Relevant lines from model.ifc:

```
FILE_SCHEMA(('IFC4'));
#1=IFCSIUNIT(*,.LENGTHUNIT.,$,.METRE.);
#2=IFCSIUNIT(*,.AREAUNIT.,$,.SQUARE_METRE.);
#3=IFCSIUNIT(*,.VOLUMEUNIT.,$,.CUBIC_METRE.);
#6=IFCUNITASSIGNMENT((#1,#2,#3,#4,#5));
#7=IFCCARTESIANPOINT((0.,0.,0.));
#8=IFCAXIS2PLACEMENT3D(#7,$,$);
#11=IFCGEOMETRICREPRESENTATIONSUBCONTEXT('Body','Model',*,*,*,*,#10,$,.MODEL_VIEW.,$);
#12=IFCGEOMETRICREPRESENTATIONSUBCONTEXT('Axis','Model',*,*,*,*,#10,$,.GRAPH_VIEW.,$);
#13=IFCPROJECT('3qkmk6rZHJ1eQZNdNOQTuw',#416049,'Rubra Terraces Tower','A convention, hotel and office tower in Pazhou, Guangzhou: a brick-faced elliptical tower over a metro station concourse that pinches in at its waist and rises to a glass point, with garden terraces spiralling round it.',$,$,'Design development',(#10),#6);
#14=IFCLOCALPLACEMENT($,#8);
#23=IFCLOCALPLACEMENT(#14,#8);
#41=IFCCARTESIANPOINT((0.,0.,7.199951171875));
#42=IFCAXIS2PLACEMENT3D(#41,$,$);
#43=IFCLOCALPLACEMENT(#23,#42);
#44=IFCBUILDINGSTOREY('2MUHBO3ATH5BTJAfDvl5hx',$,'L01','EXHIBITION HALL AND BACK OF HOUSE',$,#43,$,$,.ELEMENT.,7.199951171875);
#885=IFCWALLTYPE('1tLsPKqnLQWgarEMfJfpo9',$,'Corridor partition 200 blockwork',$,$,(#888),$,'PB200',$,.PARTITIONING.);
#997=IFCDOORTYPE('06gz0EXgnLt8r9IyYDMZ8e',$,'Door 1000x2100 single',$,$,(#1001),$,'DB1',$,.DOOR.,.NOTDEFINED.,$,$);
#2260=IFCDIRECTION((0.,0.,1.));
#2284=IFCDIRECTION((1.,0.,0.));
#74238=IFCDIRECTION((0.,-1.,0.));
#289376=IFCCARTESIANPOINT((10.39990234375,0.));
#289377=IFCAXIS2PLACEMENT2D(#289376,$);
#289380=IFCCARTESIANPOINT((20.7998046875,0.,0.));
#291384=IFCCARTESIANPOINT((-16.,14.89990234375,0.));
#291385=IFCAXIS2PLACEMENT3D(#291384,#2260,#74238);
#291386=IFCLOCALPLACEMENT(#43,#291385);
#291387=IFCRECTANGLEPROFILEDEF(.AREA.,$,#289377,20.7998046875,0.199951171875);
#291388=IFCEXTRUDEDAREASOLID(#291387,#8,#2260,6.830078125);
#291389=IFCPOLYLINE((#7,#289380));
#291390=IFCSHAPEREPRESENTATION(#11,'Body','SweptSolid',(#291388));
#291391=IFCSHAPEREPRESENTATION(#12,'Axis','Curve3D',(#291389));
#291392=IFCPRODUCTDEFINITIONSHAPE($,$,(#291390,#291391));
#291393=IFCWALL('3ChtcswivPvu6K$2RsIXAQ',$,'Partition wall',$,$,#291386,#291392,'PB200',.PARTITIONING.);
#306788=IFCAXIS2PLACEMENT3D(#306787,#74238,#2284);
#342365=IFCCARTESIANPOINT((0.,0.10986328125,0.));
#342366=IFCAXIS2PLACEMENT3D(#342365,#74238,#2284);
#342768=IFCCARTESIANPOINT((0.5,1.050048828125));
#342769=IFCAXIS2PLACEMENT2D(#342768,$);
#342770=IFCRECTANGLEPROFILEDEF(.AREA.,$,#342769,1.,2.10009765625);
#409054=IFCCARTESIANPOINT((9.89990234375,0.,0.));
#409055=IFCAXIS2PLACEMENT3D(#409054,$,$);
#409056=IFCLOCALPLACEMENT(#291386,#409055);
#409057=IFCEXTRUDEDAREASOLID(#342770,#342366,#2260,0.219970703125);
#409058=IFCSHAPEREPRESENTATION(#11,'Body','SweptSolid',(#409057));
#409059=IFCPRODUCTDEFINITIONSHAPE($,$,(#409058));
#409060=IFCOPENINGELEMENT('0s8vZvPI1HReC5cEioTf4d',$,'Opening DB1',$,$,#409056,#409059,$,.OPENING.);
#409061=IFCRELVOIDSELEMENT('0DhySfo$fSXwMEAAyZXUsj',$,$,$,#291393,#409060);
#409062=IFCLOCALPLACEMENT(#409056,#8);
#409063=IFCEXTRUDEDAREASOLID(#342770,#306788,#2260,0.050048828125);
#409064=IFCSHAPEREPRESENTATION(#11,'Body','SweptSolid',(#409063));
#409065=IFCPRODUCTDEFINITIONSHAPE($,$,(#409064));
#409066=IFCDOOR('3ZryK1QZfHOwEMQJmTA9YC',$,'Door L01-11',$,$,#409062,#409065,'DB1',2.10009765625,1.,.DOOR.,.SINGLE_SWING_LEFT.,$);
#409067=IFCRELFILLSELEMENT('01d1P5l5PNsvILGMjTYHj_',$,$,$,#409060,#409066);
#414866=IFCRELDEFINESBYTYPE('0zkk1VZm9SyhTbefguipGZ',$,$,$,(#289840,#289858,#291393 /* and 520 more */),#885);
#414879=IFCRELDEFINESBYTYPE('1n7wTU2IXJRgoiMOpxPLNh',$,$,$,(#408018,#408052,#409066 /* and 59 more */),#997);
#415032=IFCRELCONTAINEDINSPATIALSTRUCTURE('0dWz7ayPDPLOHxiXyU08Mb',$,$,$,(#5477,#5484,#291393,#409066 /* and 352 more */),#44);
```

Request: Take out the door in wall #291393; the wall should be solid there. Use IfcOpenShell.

```python
import ifcopenshell
import ifcopenshell.api.feature
import ifcopenshell.api.root
import ifcopenshell.geom
import ifcopenshell.util.shape

model = ifcopenshell.open("model.ifc")
settings = ifcopenshell.geom.settings()


def volume(element):
    """Net volume in cubic metres, openings subtracted."""
    shape = ifcopenshell.geom.create_shape(settings, element)
    return ifcopenshell.util.shape.get_volume(shape.geometry)


door = model.by_guid("3ZryK1QZfHOwEMQJmTA9YC")
opening = door.FillsVoids[0].RelatingOpeningElement
wall = opening.VoidsElements[0].RelatingBuildingElement
before = volume(wall)

ifcopenshell.api.root.remove_product(model, product=door)
ifcopenshell.api.feature.remove_feature(model, feature=opening)

after = volume(wall)

print(f"wall volume {before:.3f} -> {after:.3f} m3")

model.write("model_rev.ifc")
```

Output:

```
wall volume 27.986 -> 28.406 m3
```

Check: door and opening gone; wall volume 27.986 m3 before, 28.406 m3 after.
